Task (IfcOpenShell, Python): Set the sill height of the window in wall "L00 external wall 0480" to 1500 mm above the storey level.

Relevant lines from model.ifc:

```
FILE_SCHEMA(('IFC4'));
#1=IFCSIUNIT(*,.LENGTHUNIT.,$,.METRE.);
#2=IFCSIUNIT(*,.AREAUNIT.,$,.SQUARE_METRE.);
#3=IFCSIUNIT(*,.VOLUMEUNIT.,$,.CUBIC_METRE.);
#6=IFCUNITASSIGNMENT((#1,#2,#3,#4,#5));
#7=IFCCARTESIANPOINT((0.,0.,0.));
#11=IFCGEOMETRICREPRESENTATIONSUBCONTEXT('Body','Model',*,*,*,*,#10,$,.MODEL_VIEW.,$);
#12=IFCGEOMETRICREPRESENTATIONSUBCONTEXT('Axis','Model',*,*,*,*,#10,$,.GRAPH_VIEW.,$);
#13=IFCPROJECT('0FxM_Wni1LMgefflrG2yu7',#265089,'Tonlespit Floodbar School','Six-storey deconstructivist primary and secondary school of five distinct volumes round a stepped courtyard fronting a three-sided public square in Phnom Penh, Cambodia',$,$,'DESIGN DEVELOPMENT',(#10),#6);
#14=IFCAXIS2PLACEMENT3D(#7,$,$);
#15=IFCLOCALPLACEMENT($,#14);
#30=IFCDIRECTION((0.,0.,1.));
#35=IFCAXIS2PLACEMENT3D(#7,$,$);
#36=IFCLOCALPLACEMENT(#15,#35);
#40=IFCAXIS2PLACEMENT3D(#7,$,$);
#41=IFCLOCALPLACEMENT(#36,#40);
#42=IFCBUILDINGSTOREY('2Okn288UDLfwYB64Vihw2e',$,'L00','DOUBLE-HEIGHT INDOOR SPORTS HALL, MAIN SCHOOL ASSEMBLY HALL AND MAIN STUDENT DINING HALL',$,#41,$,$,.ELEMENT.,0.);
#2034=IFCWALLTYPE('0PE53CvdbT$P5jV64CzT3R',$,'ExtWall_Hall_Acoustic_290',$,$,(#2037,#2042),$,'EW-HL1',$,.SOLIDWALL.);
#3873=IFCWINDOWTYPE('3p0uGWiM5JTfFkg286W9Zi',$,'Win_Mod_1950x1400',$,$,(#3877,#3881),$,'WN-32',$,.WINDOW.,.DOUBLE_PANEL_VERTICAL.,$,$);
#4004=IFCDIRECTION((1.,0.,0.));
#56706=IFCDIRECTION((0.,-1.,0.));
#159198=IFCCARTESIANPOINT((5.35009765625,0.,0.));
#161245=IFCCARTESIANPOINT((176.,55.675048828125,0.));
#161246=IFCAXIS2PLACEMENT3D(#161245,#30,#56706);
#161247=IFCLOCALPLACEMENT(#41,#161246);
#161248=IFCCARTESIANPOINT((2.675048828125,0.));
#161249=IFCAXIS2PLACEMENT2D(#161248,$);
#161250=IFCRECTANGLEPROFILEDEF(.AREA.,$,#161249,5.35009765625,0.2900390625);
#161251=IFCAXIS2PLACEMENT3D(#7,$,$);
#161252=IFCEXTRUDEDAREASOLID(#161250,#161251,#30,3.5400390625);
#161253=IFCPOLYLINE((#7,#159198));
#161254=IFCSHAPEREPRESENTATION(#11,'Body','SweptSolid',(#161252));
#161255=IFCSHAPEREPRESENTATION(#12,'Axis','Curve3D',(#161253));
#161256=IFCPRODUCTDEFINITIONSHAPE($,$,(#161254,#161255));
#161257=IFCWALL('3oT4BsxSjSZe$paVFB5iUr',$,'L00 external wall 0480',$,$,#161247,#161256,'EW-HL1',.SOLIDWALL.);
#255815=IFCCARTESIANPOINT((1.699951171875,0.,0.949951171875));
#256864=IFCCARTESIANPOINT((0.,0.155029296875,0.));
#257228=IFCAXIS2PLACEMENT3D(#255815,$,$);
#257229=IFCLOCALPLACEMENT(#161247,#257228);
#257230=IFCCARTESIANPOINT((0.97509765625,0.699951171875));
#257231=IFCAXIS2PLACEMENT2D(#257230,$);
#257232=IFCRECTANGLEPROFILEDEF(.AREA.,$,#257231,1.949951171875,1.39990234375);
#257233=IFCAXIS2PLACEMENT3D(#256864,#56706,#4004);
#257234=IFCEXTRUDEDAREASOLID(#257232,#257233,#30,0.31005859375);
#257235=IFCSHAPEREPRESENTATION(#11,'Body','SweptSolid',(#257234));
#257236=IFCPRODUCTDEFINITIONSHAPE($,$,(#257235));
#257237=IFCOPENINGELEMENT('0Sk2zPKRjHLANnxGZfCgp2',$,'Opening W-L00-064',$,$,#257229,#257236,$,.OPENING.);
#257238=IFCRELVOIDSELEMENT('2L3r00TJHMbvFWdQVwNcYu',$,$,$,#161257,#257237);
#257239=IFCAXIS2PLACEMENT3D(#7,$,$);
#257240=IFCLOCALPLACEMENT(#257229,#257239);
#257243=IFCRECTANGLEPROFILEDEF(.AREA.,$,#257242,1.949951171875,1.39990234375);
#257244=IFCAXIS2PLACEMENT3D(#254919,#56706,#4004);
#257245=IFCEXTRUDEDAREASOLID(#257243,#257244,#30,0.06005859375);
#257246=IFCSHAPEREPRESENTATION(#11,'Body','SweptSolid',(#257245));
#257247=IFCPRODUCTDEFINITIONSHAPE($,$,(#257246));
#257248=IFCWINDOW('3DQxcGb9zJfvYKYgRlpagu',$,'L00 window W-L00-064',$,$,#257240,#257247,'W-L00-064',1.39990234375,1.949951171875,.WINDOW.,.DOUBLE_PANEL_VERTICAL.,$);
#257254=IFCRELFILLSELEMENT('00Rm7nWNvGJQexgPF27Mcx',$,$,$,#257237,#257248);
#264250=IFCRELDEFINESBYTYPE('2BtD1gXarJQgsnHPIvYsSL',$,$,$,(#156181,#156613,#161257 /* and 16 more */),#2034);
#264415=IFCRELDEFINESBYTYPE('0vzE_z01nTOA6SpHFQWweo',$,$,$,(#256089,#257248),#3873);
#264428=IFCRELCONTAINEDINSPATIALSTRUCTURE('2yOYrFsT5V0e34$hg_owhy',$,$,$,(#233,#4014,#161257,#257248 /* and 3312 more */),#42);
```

```python
import numpy as np
import ifcopenshell
import ifcopenshell.api.geometry
import ifcopenshell.geom
import ifcopenshell.util.element
import ifcopenshell.util.placement
import ifcopenshell.util.shape
import ifcopenshell.util.unit

model = ifcopenshell.open("model.ifc")
unit_scale = ifcopenshell.util.unit.calculate_unit_scale(model)

window = model.by_guid("3DQxcGb9zJfvYKYgRlpagu")
opening = window.FillsVoids[0].RelatingOpeningElement
storey = ifcopenshell.util.element.get_container(window, ifc_class="IfcBuildingStorey")
level = ifcopenshell.util.placement.get_local_placement(storey.ObjectPlacement)[2, 3]

# The opening's origin need not be at the sill, so measure its lowest point.
shape = ifcopenshell.geom.create_shape(ifcopenshell.geom.settings(), opening)
bottom = ifcopenshell.util.shape.get_shape_bottom_elevation(shape, shape.geometry) / unit_scale
dz = level + 1.5 / unit_scale - bottom

shift = np.array([0.0, 0.0, dz])
# The window is placed relative to its opening, so it follows when the opening moves.
matrix = ifcopenshell.util.placement.get_local_placement(opening.ObjectPlacement)
matrix[:3, 3] += shift
ifcopenshell.api.geometry.edit_object_placement(
    model, product=opening, matrix=matrix, is_si=False, should_transform_children=True
)

print(f"moved by {dz * unit_scale:+.3f} m")

model.write("model_updated.ifc")
```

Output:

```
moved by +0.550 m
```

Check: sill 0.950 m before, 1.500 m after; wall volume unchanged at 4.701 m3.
